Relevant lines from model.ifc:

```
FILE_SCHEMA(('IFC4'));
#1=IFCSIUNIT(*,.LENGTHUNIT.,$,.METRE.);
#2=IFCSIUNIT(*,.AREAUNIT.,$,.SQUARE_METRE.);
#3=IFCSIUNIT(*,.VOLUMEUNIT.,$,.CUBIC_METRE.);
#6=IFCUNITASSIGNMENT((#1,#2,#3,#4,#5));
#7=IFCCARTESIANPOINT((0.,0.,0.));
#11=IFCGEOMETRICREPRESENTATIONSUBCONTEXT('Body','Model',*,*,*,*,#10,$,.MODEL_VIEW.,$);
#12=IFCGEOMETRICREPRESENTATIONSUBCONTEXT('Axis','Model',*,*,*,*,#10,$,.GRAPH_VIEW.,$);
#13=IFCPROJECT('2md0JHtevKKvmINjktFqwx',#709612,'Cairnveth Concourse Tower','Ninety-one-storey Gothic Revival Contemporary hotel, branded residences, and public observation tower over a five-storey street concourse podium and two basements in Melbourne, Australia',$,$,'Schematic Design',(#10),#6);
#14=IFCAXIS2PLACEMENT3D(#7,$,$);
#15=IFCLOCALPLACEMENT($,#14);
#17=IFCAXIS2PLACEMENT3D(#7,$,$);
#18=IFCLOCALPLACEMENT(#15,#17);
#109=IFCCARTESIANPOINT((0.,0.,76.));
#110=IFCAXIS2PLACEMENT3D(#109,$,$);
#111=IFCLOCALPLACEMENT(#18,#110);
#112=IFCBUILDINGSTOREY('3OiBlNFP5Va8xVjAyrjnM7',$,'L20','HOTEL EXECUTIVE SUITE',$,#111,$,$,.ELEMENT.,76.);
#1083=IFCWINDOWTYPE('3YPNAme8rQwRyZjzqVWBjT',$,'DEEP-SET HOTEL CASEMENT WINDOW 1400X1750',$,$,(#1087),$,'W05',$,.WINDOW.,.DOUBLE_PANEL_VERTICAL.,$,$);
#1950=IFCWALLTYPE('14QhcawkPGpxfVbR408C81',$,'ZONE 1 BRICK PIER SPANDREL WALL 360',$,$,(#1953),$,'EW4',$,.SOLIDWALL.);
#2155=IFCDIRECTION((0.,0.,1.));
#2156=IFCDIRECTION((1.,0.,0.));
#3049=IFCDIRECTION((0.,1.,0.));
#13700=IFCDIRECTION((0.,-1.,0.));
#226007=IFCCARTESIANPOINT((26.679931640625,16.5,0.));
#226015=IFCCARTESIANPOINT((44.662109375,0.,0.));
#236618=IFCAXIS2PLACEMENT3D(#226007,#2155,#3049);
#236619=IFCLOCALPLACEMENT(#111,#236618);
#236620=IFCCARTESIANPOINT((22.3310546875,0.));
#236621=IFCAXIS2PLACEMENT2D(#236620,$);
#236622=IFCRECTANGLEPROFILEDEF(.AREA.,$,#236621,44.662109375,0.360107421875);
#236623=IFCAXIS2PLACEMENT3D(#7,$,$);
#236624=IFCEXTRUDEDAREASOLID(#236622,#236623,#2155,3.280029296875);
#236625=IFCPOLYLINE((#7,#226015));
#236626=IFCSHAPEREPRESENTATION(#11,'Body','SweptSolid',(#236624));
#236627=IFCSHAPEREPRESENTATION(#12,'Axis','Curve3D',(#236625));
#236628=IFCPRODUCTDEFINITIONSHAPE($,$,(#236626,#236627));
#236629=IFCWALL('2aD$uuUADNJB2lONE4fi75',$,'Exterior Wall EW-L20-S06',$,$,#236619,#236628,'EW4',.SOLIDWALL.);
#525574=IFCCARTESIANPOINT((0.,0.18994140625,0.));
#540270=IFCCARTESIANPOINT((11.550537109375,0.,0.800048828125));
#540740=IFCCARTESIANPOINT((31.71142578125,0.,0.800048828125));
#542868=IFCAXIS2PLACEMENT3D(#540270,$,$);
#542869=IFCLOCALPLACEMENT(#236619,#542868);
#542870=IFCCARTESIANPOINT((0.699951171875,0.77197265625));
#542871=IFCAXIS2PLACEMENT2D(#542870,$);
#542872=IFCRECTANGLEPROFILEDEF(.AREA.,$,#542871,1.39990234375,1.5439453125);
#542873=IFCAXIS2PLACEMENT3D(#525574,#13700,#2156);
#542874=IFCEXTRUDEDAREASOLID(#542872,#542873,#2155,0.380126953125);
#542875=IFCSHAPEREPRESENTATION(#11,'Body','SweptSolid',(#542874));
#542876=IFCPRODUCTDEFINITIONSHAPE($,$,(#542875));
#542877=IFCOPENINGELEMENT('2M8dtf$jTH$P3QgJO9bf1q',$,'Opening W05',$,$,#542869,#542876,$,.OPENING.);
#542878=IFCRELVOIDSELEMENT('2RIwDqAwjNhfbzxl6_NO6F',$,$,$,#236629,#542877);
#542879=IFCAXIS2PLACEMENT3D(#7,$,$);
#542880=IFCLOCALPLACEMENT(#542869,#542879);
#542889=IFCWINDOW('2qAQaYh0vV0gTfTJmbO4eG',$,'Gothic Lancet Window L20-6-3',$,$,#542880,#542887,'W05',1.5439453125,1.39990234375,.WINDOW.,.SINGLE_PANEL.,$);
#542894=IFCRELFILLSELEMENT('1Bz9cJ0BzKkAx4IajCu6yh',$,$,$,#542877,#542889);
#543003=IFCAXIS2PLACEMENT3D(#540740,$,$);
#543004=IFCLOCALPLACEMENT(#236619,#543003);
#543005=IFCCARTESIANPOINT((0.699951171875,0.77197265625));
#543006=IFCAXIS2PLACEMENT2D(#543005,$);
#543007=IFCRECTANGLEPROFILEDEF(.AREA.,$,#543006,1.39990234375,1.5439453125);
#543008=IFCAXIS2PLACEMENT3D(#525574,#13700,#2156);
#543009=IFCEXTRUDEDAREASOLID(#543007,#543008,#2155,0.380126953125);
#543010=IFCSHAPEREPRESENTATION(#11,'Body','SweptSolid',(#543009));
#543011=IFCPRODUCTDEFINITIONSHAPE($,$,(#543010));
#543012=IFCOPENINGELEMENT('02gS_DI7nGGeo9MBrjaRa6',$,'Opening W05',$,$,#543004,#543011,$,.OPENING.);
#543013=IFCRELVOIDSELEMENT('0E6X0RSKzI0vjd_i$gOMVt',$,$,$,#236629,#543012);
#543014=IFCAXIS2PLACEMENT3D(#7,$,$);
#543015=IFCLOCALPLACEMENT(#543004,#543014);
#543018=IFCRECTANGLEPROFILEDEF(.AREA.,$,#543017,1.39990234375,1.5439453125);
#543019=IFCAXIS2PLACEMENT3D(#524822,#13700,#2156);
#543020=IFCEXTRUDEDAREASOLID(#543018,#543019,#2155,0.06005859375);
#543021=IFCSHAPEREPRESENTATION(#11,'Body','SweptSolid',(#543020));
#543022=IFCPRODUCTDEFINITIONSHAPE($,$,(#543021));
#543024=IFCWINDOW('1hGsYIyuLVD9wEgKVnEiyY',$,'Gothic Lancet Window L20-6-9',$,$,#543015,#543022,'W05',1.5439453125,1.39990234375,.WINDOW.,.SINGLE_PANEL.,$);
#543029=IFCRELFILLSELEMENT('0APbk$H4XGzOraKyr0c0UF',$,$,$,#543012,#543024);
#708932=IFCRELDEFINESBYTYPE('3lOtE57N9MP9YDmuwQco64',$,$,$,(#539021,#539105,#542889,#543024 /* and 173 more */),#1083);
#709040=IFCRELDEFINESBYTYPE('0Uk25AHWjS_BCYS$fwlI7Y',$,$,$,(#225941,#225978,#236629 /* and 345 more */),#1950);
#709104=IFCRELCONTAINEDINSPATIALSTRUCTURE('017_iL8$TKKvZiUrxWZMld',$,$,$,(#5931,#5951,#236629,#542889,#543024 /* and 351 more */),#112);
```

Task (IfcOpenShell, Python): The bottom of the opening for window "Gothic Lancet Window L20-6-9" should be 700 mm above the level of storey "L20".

```python
import numpy as np
import ifcopenshell
import ifcopenshell.api.geometry
import ifcopenshell.geom
import ifcopenshell.util.element
import ifcopenshell.util.placement
import ifcopenshell.util.shape
import ifcopenshell.util.unit

model = ifcopenshell.open("model.ifc")
unit_scale = ifcopenshell.util.unit.calculate_unit_scale(model)

window = model.by_guid("1hGsYIyuLVD9wEgKVnEiyY")
opening = window.FillsVoids[0].RelatingOpeningElement
storey = ifcopenshell.util.element.get_container(window, ifc_class="IfcBuildingStorey")
level = ifcopenshell.util.placement.get_local_placement(storey.ObjectPlacement)[2, 3]

# The opening's origin need not be at the sill, so measure its lowest point.
shape = ifcopenshell.geom.create_shape(ifcopenshell.geom.settings(), opening)
bottom = ifcopenshell.util.shape.get_shape_bottom_elevation(shape, shape.geometry) / unit_scale
dz = level + 0.7 / unit_scale - bottom

shift = np.array([0.0, 0.0, dz])
# The window is placed relative to its opening, so it follows when the opening moves.
matrix = ifcopenshell.util.placement.get_local_placement(opening.ObjectPlacement)
matrix[:3, 3] += shift
ifcopenshell.api.geometry.edit_object_placement(
    model, product=opening, matrix=matrix, is_si=False, should_transform_children=True
)

print(f"moved by {dz * unit_scale:+.3f} m")

model.write("model_v2.ifc")
```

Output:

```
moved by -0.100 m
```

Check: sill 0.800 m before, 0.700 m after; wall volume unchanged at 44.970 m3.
